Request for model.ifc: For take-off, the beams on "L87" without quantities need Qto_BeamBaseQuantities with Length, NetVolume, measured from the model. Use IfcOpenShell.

First a look at what the model holds.

```python
import ifcopenshell
import ifcopenshell.util.element
import ifcopenshell.util.unit

model = ifcopenshell.open("model.ifc")
print(model.schema)
for unit_type in ("LENGTHUNIT", "AREAUNIT", "VOLUMEUNIT"):
    print(unit_type, ifcopenshell.util.unit.calculate_unit_scale(model, unit_type))
storey = next(s for s in model.by_type("IfcBuildingStorey") if s.Name == "L87")
beams = [e for e in ifcopenshell.util.element.get_decomposition(storey) if e.is_a("IfcBeam")]
for e in sorted(beams, key=lambda e: e.id()):
    print(e.id(), e.is_a(), e.Name, list(ifcopenshell.util.element.get_psets(e, qtos_only=True)), sep=" | ")
```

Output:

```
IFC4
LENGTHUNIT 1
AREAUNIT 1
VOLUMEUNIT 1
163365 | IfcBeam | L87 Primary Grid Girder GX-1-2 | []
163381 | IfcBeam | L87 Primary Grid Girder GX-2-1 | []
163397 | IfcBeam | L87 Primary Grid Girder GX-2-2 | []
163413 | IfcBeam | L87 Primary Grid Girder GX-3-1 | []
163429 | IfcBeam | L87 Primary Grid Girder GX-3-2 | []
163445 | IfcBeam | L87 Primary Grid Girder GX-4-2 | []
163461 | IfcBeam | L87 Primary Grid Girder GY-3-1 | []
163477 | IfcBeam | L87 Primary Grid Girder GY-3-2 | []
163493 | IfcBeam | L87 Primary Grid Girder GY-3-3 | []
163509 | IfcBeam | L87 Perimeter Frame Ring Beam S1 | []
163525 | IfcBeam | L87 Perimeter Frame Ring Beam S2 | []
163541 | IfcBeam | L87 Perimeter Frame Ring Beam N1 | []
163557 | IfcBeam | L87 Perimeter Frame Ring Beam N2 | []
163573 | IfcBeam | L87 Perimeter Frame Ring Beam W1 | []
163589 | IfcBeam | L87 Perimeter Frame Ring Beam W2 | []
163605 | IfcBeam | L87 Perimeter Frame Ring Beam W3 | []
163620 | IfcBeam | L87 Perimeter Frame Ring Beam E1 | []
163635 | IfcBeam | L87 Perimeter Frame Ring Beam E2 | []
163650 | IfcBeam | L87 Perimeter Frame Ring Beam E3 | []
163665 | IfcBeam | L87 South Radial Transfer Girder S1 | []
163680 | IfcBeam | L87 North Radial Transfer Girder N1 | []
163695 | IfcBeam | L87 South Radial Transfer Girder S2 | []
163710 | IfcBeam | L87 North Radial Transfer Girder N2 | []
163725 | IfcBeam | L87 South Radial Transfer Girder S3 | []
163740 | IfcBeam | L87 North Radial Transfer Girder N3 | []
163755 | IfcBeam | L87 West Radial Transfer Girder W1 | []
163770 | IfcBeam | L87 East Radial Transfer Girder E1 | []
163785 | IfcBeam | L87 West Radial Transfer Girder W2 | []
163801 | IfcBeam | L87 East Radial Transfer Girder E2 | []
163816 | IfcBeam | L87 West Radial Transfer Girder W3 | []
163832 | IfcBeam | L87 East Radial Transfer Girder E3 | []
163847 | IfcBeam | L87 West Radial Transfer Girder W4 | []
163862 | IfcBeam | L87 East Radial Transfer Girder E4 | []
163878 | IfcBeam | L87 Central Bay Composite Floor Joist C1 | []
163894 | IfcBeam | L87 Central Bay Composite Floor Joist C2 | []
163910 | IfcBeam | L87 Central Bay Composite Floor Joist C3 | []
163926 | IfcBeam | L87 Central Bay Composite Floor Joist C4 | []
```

```python
import ifcopenshell
import ifcopenshell.api.pset
import ifcopenshell.geom
import ifcopenshell.util.element
import ifcopenshell.util.shape
import ifcopenshell.util.unit

model = ifcopenshell.open("model.ifc")
unit_scale = ifcopenshell.util.unit.calculate_unit_scale(model)
volume_scale = ifcopenshell.util.unit.calculate_unit_scale(model, "VOLUMEUNIT")
settings = ifcopenshell.geom.settings()

storey = next(s for s in model.by_type("IfcBuildingStorey") if s.Name == "L87")
beams = [e for e in ifcopenshell.util.element.get_decomposition(storey) if e.is_a("IfcBeam")]

for e in sorted(beams, key=lambda e: e.id()):
    if ifcopenshell.util.element.get_psets(e, qtos_only=True, should_inherit=False):
        continue
    # Geometry comes back in metres, in the element's own axes.
    shape = ifcopenshell.geom.create_shape(settings, e)
    values = {
        "Length": ifcopenshell.util.shape.get_max_xyz(shape.geometry) / unit_scale,
        "NetVolume": ifcopenshell.util.shape.get_volume(shape.geometry) / volume_scale,
    }
    qto = ifcopenshell.api.pset.add_qto(model, product=e, name="Qto_BeamBaseQuantities")
    ifcopenshell.api.pset.edit_qto(model, qto=qto, properties=values)
    print(e.id(), {k: round(v, 3) for k, v in values.items()})

model.write("model-out.ifc")
```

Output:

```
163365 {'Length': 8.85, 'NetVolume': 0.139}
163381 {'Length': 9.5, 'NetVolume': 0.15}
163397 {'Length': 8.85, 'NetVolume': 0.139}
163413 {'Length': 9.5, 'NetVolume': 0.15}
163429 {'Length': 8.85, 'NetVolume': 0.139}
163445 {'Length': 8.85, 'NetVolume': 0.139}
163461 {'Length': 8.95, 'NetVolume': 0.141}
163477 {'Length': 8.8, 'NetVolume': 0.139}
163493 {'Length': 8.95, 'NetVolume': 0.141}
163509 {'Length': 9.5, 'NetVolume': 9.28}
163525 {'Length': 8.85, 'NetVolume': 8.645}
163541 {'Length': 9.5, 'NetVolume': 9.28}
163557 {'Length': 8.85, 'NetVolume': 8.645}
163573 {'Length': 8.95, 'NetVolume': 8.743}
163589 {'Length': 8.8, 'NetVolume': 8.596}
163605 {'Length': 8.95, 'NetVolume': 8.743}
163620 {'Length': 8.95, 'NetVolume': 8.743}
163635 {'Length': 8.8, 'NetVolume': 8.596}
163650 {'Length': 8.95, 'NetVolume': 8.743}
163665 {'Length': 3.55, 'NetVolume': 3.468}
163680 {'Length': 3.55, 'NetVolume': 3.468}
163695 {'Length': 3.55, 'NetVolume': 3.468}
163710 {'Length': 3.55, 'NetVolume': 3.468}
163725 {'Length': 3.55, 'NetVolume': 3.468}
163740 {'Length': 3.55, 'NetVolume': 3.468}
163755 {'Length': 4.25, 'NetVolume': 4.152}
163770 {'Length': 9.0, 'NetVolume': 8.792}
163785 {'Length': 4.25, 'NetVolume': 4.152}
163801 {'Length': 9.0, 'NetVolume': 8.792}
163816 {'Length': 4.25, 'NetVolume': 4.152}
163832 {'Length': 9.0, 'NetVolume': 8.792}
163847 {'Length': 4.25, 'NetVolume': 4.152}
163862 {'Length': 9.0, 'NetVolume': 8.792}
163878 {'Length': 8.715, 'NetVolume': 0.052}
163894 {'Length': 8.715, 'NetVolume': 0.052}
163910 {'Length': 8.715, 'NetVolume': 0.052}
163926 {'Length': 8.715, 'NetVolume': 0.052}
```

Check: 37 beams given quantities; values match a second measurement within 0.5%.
